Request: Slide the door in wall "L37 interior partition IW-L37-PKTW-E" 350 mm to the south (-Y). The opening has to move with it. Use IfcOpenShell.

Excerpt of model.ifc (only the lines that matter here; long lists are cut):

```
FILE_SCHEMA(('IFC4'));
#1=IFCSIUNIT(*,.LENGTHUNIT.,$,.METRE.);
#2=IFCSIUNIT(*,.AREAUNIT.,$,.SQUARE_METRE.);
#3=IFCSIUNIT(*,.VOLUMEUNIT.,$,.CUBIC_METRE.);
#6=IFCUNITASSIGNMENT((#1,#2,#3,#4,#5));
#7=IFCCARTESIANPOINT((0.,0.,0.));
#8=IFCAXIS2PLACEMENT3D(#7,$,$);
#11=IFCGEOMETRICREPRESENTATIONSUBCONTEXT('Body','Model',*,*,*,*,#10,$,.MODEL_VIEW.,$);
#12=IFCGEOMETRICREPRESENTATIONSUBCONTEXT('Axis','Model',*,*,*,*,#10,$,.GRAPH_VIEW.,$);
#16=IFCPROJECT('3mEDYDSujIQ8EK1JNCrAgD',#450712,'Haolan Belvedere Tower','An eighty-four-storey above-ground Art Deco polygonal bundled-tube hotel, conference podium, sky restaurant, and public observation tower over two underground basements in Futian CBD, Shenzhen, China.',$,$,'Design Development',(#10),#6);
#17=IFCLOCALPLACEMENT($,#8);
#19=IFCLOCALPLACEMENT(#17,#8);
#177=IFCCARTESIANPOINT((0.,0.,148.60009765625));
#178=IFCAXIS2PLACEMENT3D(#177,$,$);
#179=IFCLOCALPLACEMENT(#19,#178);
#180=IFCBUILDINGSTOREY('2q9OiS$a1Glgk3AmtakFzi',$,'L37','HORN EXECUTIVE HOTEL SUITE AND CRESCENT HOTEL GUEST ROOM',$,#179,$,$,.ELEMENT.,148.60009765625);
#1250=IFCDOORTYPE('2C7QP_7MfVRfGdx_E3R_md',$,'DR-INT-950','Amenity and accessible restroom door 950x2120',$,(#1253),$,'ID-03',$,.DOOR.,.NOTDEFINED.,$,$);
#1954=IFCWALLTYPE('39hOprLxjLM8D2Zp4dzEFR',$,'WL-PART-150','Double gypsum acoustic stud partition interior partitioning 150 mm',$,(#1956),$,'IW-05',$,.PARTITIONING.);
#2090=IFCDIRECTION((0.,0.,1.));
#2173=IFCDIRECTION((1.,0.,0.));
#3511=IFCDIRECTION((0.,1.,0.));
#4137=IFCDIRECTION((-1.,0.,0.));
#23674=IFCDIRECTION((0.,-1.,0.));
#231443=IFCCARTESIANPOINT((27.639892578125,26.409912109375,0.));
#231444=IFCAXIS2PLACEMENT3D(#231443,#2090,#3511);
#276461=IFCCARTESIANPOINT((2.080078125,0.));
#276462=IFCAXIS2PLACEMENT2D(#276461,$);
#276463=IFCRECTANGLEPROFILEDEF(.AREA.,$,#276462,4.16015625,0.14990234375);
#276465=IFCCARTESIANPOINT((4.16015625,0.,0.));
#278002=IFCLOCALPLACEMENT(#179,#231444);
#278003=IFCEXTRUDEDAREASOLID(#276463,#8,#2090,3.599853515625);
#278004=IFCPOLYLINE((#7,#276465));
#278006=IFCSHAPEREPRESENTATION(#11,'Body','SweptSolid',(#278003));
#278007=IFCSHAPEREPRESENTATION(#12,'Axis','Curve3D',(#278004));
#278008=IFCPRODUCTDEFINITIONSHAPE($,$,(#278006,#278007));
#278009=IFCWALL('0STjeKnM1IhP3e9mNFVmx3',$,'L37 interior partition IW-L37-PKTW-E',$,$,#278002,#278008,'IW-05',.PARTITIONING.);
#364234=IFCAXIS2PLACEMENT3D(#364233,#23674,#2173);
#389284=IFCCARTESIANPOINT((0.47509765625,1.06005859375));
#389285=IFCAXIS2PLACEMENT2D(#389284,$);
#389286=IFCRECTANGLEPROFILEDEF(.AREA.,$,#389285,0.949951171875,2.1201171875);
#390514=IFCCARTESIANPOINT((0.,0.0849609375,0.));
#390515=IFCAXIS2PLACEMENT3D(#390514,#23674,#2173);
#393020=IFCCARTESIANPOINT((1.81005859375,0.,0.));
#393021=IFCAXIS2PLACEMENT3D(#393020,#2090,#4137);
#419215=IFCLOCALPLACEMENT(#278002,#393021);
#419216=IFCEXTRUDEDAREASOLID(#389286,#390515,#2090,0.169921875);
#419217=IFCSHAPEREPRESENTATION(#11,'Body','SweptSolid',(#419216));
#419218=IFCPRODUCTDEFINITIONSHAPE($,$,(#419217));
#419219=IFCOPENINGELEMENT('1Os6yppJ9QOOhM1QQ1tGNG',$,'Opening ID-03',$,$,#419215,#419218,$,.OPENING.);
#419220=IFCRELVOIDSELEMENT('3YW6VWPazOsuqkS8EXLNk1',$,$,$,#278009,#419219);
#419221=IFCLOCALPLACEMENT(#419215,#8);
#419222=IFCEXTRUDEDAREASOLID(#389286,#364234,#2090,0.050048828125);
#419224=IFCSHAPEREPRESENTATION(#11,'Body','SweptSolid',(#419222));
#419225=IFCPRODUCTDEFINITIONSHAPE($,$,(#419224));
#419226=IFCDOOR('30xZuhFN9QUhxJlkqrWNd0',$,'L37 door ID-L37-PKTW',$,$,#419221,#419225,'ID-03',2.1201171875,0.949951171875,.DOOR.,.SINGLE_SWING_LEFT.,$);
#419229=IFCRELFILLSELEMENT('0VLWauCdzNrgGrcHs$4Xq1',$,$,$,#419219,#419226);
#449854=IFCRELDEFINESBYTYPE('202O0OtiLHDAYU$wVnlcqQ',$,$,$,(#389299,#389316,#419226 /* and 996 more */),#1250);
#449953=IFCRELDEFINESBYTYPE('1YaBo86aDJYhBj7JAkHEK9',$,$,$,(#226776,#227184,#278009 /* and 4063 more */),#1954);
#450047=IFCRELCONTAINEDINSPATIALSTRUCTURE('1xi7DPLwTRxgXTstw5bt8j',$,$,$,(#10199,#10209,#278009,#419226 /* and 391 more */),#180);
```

```python
import ifcopenshell
import ifcopenshell.api.geometry
import ifcopenshell.util.placement
import ifcopenshell.util.unit

model = ifcopenshell.open("model.ifc")
unit_scale = ifcopenshell.util.unit.calculate_unit_scale(model)

door = model.by_guid("30xZuhFN9QUhxJlkqrWNd0")
opening = door.FillsVoids[0].RelatingOpeningElement
wall = opening.VoidsElements[0].RelatingBuildingElement

wall_matrix = ifcopenshell.util.placement.get_local_placement(wall.ObjectPlacement)
shift = wall_matrix[:3, 0] * -0.35 / unit_scale
before = ifcopenshell.util.placement.get_local_placement(door.ObjectPlacement)[:3, 3].copy()

# The door is placed relative to its opening, so it follows when the opening moves.
matrix = ifcopenshell.util.placement.get_local_placement(opening.ObjectPlacement)
matrix[:3, 3] += shift
ifcopenshell.api.geometry.edit_object_placement(
    model, product=opening, matrix=matrix, is_si=False, should_transform_children=True
)

after = ifcopenshell.util.placement.get_local_placement(door.ObjectPlacement)[:3, 3]
print("door moved by", (after - before).round(3) + 0.0)

model.write("model_updated.ifc")
```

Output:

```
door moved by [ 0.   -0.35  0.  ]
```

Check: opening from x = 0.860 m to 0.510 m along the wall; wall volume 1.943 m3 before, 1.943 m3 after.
